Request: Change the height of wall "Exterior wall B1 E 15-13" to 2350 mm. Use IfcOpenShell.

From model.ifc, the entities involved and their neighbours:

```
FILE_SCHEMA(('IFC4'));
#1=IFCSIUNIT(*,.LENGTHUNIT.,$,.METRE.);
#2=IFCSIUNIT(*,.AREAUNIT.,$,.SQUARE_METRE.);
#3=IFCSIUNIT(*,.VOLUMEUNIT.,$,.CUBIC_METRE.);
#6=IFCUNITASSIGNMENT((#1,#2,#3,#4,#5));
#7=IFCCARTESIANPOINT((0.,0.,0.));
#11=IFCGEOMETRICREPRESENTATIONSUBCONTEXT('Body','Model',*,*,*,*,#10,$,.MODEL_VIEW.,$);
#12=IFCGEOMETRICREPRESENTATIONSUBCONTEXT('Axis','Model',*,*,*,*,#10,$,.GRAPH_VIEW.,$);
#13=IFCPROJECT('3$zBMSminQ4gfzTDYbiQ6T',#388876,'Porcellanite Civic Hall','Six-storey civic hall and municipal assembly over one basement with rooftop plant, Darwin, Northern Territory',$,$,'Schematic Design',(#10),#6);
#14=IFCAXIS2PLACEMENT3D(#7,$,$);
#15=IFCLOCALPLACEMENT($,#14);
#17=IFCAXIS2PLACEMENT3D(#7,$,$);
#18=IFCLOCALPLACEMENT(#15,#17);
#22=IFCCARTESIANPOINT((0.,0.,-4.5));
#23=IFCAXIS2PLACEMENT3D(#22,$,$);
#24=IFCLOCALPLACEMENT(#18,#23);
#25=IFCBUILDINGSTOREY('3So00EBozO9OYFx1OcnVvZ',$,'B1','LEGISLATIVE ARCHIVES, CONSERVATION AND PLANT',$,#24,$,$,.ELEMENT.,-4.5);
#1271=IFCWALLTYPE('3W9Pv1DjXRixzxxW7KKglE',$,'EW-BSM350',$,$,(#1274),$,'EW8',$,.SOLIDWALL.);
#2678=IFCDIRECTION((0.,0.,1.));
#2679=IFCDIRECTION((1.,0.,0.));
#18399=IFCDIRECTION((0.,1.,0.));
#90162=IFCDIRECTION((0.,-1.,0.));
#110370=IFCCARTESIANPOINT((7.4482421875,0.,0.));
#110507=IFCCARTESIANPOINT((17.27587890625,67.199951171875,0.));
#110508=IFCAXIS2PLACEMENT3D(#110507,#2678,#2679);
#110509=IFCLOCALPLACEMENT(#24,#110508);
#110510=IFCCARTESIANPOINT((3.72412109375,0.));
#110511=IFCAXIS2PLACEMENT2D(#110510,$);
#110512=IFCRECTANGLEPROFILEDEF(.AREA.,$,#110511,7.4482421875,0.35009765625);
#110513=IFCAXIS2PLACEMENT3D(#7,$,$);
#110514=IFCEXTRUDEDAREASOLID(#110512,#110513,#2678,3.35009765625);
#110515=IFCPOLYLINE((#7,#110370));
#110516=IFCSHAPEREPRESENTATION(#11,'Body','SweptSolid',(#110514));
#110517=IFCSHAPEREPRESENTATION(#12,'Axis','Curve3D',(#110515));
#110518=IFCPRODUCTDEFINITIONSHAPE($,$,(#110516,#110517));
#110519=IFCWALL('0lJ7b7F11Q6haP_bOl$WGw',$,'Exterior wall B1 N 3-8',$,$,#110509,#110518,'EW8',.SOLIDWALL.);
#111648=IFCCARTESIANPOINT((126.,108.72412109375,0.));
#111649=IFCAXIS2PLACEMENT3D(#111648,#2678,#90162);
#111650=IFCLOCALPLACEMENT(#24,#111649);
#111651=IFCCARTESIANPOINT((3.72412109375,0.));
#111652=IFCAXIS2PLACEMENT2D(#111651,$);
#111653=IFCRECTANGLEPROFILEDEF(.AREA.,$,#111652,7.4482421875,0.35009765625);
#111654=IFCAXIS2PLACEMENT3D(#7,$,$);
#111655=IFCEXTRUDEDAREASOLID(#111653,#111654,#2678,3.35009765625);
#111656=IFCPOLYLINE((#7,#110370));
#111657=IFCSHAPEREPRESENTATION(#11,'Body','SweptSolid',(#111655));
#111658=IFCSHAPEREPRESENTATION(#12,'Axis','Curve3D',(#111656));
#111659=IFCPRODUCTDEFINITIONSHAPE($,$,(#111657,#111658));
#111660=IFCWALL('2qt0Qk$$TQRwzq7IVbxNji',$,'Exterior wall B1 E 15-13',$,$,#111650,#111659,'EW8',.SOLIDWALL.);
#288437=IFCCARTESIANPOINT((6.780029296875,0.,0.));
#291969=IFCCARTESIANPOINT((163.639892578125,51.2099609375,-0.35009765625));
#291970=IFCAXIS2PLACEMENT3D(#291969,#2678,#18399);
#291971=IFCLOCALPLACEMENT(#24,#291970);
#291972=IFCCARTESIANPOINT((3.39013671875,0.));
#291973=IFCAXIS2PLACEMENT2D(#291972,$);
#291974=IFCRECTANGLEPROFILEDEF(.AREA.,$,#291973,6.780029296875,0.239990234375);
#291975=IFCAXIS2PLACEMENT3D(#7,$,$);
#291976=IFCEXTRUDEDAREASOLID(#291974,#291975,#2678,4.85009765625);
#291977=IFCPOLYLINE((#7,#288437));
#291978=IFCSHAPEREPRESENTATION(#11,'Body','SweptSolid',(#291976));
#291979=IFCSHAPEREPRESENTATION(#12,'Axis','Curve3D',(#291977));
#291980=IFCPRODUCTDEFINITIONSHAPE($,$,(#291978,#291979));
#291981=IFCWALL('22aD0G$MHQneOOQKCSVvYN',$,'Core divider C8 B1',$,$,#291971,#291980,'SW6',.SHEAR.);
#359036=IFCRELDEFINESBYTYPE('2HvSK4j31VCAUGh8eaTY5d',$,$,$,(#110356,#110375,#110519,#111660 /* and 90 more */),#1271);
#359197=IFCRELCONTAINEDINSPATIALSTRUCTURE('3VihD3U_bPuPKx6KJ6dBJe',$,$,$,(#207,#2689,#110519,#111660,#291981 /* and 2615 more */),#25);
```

```python
import ifcopenshell
import ifcopenshell.geom
import ifcopenshell.util.representation
import ifcopenshell.util.shape
import ifcopenshell.util.unit

model = ifcopenshell.open("model.ifc")
unit_scale = ifcopenshell.util.unit.calculate_unit_scale(model)
settings = ifcopenshell.geom.settings()


def volume(element):
    """Net volume in cubic metres, openings subtracted."""
    shape = ifcopenshell.geom.create_shape(settings, element)
    return ifcopenshell.util.shape.get_volume(shape.geometry)


wall = model.by_guid("2qt0Qk$$TQRwzq7IVbxNji")
before = volume(wall)

body = ifcopenshell.util.representation.get_representation(wall, "Model", "Body")
solid = body.Items[0]
old_height = solid.Depth
solid.Depth = 2.35 / unit_scale
after = volume(wall)

print(f"height {old_height:g} -> {solid.Depth:g}, volume {before:.3f} -> {after:.3f} m3")

model.write("model_rev.ifc")
```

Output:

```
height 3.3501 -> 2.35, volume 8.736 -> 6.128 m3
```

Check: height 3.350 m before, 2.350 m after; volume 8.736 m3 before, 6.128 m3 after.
